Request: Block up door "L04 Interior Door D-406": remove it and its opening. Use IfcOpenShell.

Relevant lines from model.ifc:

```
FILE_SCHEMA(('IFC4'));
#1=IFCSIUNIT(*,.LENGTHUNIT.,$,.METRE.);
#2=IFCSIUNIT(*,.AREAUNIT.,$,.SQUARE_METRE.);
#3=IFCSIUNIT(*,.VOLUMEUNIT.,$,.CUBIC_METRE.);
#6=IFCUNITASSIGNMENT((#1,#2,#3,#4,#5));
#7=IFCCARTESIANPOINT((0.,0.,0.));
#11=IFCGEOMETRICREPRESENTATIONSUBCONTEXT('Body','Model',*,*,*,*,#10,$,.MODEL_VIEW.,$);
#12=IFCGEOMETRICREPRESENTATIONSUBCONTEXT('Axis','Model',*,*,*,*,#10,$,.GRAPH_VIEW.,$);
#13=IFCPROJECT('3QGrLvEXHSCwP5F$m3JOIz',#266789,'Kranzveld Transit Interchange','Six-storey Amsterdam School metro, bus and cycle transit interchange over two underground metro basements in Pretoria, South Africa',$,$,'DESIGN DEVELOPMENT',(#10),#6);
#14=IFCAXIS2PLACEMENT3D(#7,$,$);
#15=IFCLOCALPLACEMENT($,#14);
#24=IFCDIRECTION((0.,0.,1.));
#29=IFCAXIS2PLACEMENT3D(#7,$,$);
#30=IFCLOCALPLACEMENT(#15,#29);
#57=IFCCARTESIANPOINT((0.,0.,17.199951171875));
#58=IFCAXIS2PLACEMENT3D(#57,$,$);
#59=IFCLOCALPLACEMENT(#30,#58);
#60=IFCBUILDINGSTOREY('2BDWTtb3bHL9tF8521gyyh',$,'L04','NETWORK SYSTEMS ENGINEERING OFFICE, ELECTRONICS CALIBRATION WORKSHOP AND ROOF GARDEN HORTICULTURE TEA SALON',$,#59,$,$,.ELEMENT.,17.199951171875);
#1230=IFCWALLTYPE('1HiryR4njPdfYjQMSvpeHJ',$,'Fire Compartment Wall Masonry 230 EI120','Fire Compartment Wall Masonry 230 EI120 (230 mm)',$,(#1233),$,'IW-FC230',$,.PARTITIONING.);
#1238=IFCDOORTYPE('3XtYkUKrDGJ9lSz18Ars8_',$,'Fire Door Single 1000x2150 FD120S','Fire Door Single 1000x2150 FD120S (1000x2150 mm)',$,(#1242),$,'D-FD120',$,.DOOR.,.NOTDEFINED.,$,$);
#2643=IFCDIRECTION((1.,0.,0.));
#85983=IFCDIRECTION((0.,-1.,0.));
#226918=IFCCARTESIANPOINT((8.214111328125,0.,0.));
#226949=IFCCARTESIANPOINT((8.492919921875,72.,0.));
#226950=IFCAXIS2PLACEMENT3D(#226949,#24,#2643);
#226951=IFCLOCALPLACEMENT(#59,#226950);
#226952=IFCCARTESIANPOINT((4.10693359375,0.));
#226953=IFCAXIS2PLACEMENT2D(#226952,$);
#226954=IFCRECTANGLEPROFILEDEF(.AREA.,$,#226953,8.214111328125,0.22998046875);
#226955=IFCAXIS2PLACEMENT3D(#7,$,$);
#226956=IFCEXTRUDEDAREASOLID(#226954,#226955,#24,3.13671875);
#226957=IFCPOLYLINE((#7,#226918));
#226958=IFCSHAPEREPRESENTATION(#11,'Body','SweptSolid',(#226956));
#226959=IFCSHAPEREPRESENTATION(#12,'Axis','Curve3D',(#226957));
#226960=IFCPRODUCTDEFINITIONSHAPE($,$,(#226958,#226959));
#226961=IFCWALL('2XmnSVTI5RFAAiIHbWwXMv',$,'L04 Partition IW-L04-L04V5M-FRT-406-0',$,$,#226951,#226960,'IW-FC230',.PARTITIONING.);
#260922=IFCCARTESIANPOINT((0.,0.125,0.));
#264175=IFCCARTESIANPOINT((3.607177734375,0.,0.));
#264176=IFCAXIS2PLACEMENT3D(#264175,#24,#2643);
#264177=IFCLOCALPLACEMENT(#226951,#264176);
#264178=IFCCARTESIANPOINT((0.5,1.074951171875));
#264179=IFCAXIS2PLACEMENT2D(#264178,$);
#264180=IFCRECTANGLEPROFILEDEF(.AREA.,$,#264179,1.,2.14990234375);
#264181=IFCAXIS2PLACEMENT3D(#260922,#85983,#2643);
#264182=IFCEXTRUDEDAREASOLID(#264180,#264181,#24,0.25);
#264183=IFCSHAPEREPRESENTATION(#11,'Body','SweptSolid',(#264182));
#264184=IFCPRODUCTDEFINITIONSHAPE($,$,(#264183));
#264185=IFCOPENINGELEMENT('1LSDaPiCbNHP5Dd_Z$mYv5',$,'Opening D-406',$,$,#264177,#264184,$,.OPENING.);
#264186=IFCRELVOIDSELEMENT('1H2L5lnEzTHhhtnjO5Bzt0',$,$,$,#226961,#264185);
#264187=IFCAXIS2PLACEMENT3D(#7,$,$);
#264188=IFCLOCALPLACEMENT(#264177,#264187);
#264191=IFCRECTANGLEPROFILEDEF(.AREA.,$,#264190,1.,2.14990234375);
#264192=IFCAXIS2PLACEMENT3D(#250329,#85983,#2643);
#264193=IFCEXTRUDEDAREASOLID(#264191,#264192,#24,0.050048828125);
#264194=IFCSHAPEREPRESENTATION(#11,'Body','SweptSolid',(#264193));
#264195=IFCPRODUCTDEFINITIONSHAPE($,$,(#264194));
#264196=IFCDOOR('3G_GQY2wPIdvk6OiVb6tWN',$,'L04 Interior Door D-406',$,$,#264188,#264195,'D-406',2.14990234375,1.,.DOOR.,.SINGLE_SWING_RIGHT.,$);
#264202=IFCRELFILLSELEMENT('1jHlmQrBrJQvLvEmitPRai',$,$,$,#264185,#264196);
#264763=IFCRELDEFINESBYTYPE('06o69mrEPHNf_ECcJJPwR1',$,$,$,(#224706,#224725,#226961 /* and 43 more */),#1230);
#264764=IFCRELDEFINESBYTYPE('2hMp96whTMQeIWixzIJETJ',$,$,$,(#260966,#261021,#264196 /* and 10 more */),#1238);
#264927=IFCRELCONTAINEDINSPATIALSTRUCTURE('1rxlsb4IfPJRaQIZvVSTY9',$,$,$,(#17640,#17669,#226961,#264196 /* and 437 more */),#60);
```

```python
import ifcopenshell
import ifcopenshell.api.feature
import ifcopenshell.api.root
import ifcopenshell.geom
import ifcopenshell.util.shape

model = ifcopenshell.open("model.ifc")
settings = ifcopenshell.geom.settings()


def volume(element):
    """Net volume in cubic metres, openings subtracted."""
    shape = ifcopenshell.geom.create_shape(settings, element)
    return ifcopenshell.util.shape.get_volume(shape.geometry)


door = model.by_guid("3G_GQY2wPIdvk6OiVb6tWN")
opening = door.FillsVoids[0].RelatingOpeningElement
wall = opening.VoidsElements[0].RelatingBuildingElement
before = volume(wall)

ifcopenshell.api.root.remove_product(model, product=door)
ifcopenshell.api.feature.remove_feature(model, feature=opening)

after = volume(wall)

print(f"wall volume {before:.3f} -> {after:.3f} m3")

model.write("model_edited.ifc")
```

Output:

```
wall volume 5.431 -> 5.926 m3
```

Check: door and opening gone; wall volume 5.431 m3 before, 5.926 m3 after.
